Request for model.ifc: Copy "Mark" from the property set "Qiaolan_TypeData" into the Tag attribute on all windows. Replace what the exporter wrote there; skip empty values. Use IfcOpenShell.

First a look at what the model holds.

```python
import ifcopenshell
import ifcopenshell.util.element

model = ifcopenshell.open("model.ifc")
print(model.schema)
windows = model.by_type("IfcWindow")
print(len(windows), "windows")
for e in windows[:8]:
    source = ifcopenshell.util.element.get_pset(e, "Qiaolan_TypeData", "Mark")
    target = e.Tag
    print(e.id(), repr(source), repr(target), sep=" | ")
```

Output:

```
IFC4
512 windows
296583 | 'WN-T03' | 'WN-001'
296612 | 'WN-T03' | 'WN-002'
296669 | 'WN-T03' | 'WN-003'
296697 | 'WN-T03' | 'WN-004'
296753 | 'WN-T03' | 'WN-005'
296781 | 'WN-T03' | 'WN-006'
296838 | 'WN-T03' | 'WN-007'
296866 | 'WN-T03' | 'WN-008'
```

```python
import ifcopenshell
import ifcopenshell.util.element

model = ifcopenshell.open("model.ifc")

count = 0
for e in model.by_type("IfcWindow"):
    value = ifcopenshell.util.element.get_pset(e, "Qiaolan_TypeData", "Mark")
    current = e.Tag
    if not value or not value.strip() or current == value:
        continue
    e.Tag = value
    count += 1

print(count, "windows updated")

model.write("model_rev.ifc")
```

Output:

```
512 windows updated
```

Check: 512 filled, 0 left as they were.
